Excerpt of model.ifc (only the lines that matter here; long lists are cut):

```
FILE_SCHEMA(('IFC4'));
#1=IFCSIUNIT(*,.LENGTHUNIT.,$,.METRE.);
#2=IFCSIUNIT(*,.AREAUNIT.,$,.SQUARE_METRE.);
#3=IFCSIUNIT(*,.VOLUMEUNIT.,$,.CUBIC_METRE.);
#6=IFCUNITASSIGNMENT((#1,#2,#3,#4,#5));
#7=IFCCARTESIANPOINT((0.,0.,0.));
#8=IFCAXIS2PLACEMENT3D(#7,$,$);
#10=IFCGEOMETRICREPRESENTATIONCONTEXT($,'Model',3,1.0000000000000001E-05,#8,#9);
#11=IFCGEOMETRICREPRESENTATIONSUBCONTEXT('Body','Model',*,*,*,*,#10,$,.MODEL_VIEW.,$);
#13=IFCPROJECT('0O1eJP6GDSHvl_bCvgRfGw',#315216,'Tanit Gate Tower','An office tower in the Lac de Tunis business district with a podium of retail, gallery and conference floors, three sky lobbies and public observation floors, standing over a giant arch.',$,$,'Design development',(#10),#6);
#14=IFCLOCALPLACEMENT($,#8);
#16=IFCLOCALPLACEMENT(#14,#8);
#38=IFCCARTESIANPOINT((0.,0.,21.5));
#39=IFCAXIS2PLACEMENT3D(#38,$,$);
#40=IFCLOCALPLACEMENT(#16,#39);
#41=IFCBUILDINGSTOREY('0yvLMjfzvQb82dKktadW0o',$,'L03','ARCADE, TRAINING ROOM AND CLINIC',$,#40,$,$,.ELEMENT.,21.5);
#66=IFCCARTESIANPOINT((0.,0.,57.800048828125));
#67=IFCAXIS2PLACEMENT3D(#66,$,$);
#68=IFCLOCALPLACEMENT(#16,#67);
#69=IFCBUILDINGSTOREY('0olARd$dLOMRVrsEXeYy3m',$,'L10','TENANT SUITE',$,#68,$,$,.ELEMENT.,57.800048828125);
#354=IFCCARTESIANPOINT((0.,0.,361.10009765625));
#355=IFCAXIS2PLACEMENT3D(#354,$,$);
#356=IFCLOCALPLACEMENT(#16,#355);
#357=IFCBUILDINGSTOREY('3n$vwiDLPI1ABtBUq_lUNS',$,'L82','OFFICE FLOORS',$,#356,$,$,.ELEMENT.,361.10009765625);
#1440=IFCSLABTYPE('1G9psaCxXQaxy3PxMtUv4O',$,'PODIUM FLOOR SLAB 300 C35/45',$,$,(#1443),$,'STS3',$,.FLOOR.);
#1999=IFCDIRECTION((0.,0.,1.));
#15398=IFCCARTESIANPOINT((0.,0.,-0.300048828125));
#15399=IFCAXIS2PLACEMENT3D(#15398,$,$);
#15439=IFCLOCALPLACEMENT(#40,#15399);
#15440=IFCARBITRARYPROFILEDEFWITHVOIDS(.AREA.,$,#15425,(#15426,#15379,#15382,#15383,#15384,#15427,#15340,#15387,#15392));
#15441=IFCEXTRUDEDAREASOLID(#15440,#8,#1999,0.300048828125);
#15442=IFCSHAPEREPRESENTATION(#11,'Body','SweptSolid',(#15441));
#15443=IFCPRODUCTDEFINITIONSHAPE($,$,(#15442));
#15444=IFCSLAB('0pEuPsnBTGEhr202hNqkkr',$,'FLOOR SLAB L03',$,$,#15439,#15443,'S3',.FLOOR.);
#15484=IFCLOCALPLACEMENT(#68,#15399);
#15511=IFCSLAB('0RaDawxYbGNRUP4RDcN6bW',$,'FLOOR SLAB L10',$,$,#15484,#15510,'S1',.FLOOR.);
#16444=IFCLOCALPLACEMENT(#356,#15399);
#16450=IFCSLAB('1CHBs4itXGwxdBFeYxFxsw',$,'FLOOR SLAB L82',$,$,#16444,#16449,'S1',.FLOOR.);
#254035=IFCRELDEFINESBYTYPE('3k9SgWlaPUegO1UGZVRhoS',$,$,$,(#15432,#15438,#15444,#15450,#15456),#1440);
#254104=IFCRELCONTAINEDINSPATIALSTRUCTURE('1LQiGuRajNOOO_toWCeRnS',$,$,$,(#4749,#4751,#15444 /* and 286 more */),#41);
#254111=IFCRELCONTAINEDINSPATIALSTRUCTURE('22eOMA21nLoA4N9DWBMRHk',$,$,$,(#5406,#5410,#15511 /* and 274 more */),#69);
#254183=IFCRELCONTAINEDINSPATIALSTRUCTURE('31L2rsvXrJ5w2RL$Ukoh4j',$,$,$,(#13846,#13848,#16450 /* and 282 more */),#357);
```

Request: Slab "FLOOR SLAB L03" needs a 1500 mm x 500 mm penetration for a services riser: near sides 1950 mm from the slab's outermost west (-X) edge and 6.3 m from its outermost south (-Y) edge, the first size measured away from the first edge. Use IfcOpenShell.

```python
import numpy as np
import ifcopenshell
import ifcopenshell.api.feature
import ifcopenshell.api.geometry
import ifcopenshell.api.root
import ifcopenshell.geom
import ifcopenshell.util.placement
import ifcopenshell.util.representation
import ifcopenshell.util.shape
import ifcopenshell.util.unit

model = ifcopenshell.open("model.ifc")
unit_scale = ifcopenshell.util.unit.calculate_unit_scale(model)
settings = ifcopenshell.geom.settings()


def volume(element):
    """Net volume in cubic metres, openings subtracted."""
    shape = ifcopenshell.geom.create_shape(settings, element)
    return ifcopenshell.util.shape.get_volume(shape.geometry)


slab = model.by_guid("0pEuPsnBTGEhr202hNqkkr")
before = volume(slab)

# Extent in the slab's own axes, in metres. The edges named are its -X and -Y sides.
slab_shape = ifcopenshell.geom.create_shape(settings, slab)
vertices = ifcopenshell.util.shape.get_vertices(slab_shape.geometry)
x_min, y_min, bottom = vertices.min(axis=0)
top = vertices[:, 2].max()

opening = ifcopenshell.api.root.create_entity(model, ifc_class="IfcOpeningElement", name="Services riser opening", predefined_type="OPENING")
context = ifcopenshell.util.representation.get_context(model, "Model", "Body", "MODEL_VIEW")
width, depth = 1.5, 0.5
outline = [(0.0, 0.0), (width, 0.0), (width, depth), (0.0, depth), (0.0, 0.0)]
# Overshoot both faces by 50 mm so the cut is clean.
shape = ifcopenshell.api.geometry.add_slab_representation(
    model, context=context, depth=top - bottom + 0.1, polyline=outline
)
ifcopenshell.api.geometry.assign_representation(model, product=opening, representation=shape)

matrix = ifcopenshell.util.placement.get_local_placement(slab.ObjectPlacement)
matrix[:, 3] = matrix @ np.append(np.array([x_min + 1.95, y_min + 6.3, bottom - 0.05]) / unit_scale, 1.0)
ifcopenshell.api.geometry.edit_object_placement(model, product=opening, matrix=matrix, is_si=False)
ifcopenshell.api.feature.add_feature(model, feature=opening, element=slab)

after = volume(slab)

print(f"slab volume {before:.3f} -> {after:.3f} m3")

model.write("model_edited.ifc")
```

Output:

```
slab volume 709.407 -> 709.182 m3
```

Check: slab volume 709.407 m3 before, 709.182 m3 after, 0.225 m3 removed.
